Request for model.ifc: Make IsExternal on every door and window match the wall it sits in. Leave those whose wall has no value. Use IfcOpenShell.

First a look at what the model holds.

```python
import ifcopenshell
import ifcopenshell.util.element

model = ifcopenshell.open("model.ifc")
print(model.schema)
seen = {}
for e in model.by_type("IfcDoor") + model.by_type("IfcWindow"):
    if not e.FillsVoids:
        continue
    host = e.FillsVoids[0].RelatingOpeningElement.VoidsElements[0].RelatingBuildingElement
    own = ifcopenshell.util.element.get_pset(e, f"Pset_{e.is_a()[3:].removesuffix('StandardCase')}Common", "IsExternal")
    wall = ifcopenshell.util.element.get_pset(host, "Pset_WallCommon", "IsExternal")
    seen[e.is_a(), own, wall] = seen.get((e.is_a(), own, wall), 0) + 1
for (cls, own, wall), count in sorted(seen.items(), key=str):
    print(count, cls, "IsExternal:", own, "| host wall:", wall)
```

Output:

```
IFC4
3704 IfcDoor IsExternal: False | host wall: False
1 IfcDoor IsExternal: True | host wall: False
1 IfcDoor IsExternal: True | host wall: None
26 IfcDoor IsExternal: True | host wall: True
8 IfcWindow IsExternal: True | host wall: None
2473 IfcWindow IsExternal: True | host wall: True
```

```python
import ifcopenshell
import ifcopenshell.api.pset
import ifcopenshell.util.element

model = ifcopenshell.open("model.ifc")

count = 0
for ifc_class, pset_name in (("IfcDoor", "Pset_DoorCommon"), ("IfcWindow", "Pset_WindowCommon")):
    for e in model.by_type(ifc_class):
        if not e.FillsVoids:
            continue
        host = e.FillsVoids[0].RelatingOpeningElement.VoidsElements[0].RelatingBuildingElement
        external = ifcopenshell.util.element.get_pset(host, "Pset_WallCommon", "IsExternal")
        if external is None or ifcopenshell.util.element.get_pset(e, pset_name, "IsExternal") == external:
            continue
        pset = ifcopenshell.api.pset.add_pset(model, product=e, name=pset_name)
        ifcopenshell.api.pset.edit_pset(model, pset=pset, properties={"IsExternal": external})
        count += 1

print(count, "updated")

model.write("model-out.ifc")
```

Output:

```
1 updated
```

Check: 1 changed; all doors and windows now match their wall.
